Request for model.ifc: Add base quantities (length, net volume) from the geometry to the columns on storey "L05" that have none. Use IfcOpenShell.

First a look at what the model holds.

```python
import ifcopenshell
import ifcopenshell.util.element
import ifcopenshell.util.unit

model = ifcopenshell.open("model.ifc")
print(model.schema)
for unit_type in ("LENGTHUNIT", "AREAUNIT", "VOLUMEUNIT"):
    print(unit_type, ifcopenshell.util.unit.calculate_unit_scale(model, unit_type))
storey = next(s for s in model.by_type("IfcBuildingStorey") if s.Name == "L05")
columns = [e for e in ifcopenshell.util.element.get_decomposition(storey) if e.is_a("IfcColumn")]
for e in sorted(columns, key=lambda e: e.id()):
    print(e.id(), e.is_a(), e.Name, list(ifcopenshell.util.element.get_psets(e, qtos_only=True)), sep=" | ")
```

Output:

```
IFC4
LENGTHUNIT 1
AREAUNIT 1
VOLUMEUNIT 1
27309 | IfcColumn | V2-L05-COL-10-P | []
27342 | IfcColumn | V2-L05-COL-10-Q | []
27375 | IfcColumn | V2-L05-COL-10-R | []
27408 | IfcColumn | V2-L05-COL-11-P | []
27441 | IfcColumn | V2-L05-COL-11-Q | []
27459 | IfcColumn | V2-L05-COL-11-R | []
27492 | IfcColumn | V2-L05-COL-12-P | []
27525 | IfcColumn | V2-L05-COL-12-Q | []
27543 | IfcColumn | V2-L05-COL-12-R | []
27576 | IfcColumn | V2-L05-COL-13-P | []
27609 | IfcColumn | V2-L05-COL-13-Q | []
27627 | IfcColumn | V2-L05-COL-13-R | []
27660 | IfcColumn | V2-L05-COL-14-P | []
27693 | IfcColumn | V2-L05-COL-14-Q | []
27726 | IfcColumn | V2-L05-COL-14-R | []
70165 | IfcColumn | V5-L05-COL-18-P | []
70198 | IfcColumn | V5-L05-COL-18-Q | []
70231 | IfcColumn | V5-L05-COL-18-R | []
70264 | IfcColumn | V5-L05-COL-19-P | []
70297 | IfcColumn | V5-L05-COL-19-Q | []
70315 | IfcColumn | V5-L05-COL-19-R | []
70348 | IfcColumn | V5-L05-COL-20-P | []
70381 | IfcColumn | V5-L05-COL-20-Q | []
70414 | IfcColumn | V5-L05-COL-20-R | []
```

```python
import ifcopenshell
import ifcopenshell.api.pset
import ifcopenshell.geom
import ifcopenshell.util.element
import ifcopenshell.util.shape
import ifcopenshell.util.unit

model = ifcopenshell.open("model.ifc")
unit_scale = ifcopenshell.util.unit.calculate_unit_scale(model)
volume_scale = ifcopenshell.util.unit.calculate_unit_scale(model, "VOLUMEUNIT")
settings = ifcopenshell.geom.settings()

storey = next(s for s in model.by_type("IfcBuildingStorey") if s.Name == "L05")
columns = [e for e in ifcopenshell.util.element.get_decomposition(storey) if e.is_a("IfcColumn")]

for e in sorted(columns, key=lambda e: e.id()):
    if ifcopenshell.util.element.get_psets(e, qtos_only=True, should_inherit=False):
        continue
    # Geometry comes back in metres, in the element's own axes.
    shape = ifcopenshell.geom.create_shape(settings, e)
    values = {
        "Length": ifcopenshell.util.shape.get_z(shape.geometry) / unit_scale,
        "NetVolume": ifcopenshell.util.shape.get_volume(shape.geometry) / volume_scale,
    }
    qto = ifcopenshell.api.pset.add_qto(model, product=e, name="Qto_ColumnBaseQuantities")
    ifcopenshell.api.pset.edit_qto(model, qto=qto, properties=values)
    print(e.id(), {k: round(v, 3) for k, v in values.items()})

model.write("model-out.ifc")
```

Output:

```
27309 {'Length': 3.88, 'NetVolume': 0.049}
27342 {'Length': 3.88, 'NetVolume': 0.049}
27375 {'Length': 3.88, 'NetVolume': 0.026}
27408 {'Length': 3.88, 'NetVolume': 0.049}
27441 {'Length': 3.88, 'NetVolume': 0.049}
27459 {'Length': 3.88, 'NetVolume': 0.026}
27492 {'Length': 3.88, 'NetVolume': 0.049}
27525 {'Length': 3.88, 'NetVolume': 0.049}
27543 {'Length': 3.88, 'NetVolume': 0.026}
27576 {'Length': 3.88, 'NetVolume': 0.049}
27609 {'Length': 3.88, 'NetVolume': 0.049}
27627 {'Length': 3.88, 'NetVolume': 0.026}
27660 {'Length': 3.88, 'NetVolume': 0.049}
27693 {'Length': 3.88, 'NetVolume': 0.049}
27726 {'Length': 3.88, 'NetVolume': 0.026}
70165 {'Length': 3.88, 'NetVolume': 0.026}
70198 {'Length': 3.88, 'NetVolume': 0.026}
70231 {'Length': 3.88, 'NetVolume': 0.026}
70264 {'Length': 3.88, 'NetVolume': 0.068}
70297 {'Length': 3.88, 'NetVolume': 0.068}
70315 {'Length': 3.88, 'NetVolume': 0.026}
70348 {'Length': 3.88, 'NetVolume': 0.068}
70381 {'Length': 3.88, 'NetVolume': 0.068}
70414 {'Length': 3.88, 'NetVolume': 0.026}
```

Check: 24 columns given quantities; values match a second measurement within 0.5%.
